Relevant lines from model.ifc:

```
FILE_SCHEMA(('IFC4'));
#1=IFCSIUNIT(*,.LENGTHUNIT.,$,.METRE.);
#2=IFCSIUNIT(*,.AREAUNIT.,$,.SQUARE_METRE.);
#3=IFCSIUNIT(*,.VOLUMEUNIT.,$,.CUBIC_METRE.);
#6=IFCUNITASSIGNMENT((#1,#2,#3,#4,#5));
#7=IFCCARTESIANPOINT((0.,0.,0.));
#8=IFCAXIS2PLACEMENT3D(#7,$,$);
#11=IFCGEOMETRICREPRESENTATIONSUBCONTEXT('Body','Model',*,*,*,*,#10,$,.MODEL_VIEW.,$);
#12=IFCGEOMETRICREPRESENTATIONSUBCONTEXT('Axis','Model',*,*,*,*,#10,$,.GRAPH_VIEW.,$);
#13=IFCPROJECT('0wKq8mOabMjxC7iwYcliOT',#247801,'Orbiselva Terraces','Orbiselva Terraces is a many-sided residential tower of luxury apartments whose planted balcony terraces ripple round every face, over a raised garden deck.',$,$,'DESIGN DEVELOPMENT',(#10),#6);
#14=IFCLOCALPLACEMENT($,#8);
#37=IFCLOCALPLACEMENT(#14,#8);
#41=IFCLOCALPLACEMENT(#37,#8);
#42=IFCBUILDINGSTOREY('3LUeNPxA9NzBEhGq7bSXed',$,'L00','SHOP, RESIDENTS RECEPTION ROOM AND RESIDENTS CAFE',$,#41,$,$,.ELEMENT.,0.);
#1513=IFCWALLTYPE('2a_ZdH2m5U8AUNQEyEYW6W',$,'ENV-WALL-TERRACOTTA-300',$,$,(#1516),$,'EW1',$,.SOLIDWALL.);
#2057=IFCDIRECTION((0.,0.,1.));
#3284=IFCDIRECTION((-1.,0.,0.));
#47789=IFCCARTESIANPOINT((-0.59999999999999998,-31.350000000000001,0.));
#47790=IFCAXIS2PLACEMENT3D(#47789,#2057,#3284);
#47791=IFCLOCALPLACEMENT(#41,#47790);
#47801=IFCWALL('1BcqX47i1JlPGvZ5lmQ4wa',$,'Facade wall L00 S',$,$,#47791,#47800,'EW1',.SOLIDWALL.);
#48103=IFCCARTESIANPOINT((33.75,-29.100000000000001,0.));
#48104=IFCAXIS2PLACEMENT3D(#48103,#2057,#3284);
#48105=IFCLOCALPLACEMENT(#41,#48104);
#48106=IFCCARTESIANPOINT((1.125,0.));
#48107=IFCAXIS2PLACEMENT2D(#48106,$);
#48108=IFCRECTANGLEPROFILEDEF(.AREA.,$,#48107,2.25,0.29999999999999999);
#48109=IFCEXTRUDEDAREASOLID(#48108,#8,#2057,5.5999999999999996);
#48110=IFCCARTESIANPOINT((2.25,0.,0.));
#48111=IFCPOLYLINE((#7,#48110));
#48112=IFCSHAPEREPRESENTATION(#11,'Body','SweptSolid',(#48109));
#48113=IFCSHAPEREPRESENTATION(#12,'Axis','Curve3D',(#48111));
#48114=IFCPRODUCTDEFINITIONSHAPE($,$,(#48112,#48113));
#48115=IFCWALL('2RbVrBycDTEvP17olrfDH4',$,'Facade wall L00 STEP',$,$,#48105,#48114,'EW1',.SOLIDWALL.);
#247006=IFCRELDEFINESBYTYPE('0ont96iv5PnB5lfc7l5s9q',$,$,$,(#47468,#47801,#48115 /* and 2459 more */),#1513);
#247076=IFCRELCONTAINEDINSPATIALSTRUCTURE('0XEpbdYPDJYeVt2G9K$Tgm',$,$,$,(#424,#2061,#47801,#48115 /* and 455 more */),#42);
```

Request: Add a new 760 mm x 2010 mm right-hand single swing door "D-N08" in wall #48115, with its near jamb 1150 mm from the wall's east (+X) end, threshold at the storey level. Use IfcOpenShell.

```python
import numpy as np
import ifcopenshell
import ifcopenshell.api.feature
import ifcopenshell.api.geometry
import ifcopenshell.api.root
import ifcopenshell.api.spatial
import ifcopenshell.geom
import ifcopenshell.util.element
import ifcopenshell.util.placement
import ifcopenshell.util.representation
import ifcopenshell.util.shape
import ifcopenshell.util.unit

model = ifcopenshell.open("model.ifc")
unit_scale = ifcopenshell.util.unit.calculate_unit_scale(model)
settings = ifcopenshell.geom.settings()


def volume(element):
    """Net volume in cubic metres, openings subtracted."""
    shape = ifcopenshell.geom.create_shape(settings, element)
    return ifcopenshell.util.shape.get_volume(shape.geometry)


wall = model.by_guid("2RbVrBycDTEvP17olrfDH4")
storey = ifcopenshell.util.element.get_container(wall, ifc_class="IfcBuildingStorey")
context = ifcopenshell.util.representation.get_context(model, "Model", "Body", "MODEL_VIEW")
before = volume(wall)

width, height, from_end, sill = 0.76, 2.01, 1.15, 0.0  # metres

# The wall runs along its own X axis, and the end named is its -X end.
wall_shape = ifcopenshell.geom.create_shape(settings, wall)
x, y, z = ifcopenshell.util.shape.get_vertices(wall_shape.geometry).T
start = x.min() + from_end
face, thickness = float(y.min()), float(y.max() - y.min())
wall_matrix = ifcopenshell.util.placement.get_local_placement(wall.ObjectPlacement)
level = ifcopenshell.util.placement.get_local_placement(storey.ObjectPlacement)[2, 3]


def in_wall(x, y):
    """Placement at x, y metres in the wall's axes, at sill height."""
    matrix = wall_matrix.copy()
    matrix[:, 3] = wall_matrix @ np.array([x / unit_scale, y / unit_scale, 0.0, 1.0])
    matrix[2, 3] = level + sill / unit_scale
    return matrix


# Opening: a box that overshoots both wall faces by 50 mm.
opening = ifcopenshell.api.root.create_entity(model, ifc_class="IfcOpeningElement", predefined_type="OPENING")
box = ifcopenshell.api.geometry.add_wall_representation(
    model, context=context, length=width, height=height, thickness=thickness + 0.1
)
ifcopenshell.api.geometry.assign_representation(model, product=opening, representation=box)
ifcopenshell.api.geometry.edit_object_placement(model, product=opening, matrix=in_wall(start, face - 0.05), is_si=False)
ifcopenshell.api.feature.add_feature(model, feature=opening, element=wall)

door = ifcopenshell.api.root.create_entity(model, ifc_class="IfcDoor", name="D-N08", predefined_type="DOOR")
door.OverallWidth, door.OverallHeight = width / unit_scale, height / unit_scale
door.OperationType = "SINGLE_SWING_RIGHT"
body = ifcopenshell.api.geometry.add_door_representation(
    model,
    context=context,
    overall_width=door.OverallWidth,
    overall_height=door.OverallHeight,
    operation_type="SINGLE_SWING_RIGHT",
    lining_properties={"LiningDepth": thickness / unit_scale, "ThresholdDepth": thickness / unit_scale},
)
ifcopenshell.api.geometry.assign_representation(model, product=door, representation=body)
ifcopenshell.api.spatial.assign_container(model, products=[door], relating_structure=storey)
ifcopenshell.api.feature.add_filling(model, opening=opening, element=door)

# The lining spans the wall, so the door starts at the wall face.
ifcopenshell.api.geometry.edit_object_placement(model, product=door, matrix=in_wall(start, face), is_si=False)

after = volume(wall)

print(f"wall volume {before:.3f} -> {after:.3f} m3")

model.write("model_edited.ifc")
```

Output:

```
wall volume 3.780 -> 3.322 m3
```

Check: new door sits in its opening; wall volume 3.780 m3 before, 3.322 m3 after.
